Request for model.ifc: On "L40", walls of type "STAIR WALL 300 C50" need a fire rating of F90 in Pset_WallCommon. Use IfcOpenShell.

First a look at what the model holds.

```python
import ifcopenshell
import ifcopenshell.util.element

model = ifcopenshell.open("model.ifc")
print(model.schema)
storey = next(s for s in model.by_type("IfcBuildingStorey") if s.Name == "L40")
walls = [e for e in ifcopenshell.util.element.get_decomposition(storey) if e.is_a("IfcWall")]
seen = {}
for e in walls:
    element_type = ifcopenshell.util.element.get_type(e)
    key = (element_type.Name if element_type != e and element_type else None, ifcopenshell.util.element.get_pset(e, "Pset_WallCommon", "FireRating"))
    seen[key] = seen.get(key, 0) + 1
for (name, value), count in sorted(seen.items(), key=str):
    print(count, "x", name, "|", value)
```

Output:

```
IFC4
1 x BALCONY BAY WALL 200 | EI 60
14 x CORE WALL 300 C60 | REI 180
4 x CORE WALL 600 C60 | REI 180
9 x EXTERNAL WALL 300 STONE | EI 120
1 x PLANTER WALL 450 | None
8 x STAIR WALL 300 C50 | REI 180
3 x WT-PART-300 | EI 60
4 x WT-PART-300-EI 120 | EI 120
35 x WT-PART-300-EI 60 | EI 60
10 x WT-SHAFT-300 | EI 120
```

```python
import ifcopenshell
import ifcopenshell.api.pset
import ifcopenshell.util.element

model = ifcopenshell.open("model.ifc")

storey = next(s for s in model.by_type("IfcBuildingStorey") if s.Name == "L40")
walls = [e for e in ifcopenshell.util.element.get_decomposition(storey) if e.is_a("IfcWall")]

count = 0
for e in walls:
    element_type = ifcopenshell.util.element.get_type(e)
    if element_type in (None, e) or element_type.Name != "STAIR WALL 300 C50":
        continue
    found = ifcopenshell.util.element.get_pset(e, "Pset_WallCommon", should_inherit=False)
    if found:
        pset = model.by_id(found["id"])
        if len(ifcopenshell.util.element.get_elements_by_pset(pset)) > 1:
            pset = ifcopenshell.api.pset.unshare_pset(model, products=[e], pset=pset)[0]
    else:
        pset = ifcopenshell.api.pset.add_pset(model, product=e, name="Pset_WallCommon")
    ifcopenshell.api.pset.edit_pset(model, pset=pset, properties={"FireRating": "F90"})
    count += 1

print(count, "walls updated")

model.write("model_edited.ifc")
```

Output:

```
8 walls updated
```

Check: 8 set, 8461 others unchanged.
